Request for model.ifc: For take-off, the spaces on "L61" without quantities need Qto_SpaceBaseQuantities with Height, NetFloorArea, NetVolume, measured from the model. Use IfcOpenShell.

First a look at what the model holds.

```python
import ifcopenshell
import ifcopenshell.util.element
import ifcopenshell.util.unit

model = ifcopenshell.open("model.ifc")
print(model.schema)
for unit_type in ("LENGTHUNIT", "AREAUNIT", "VOLUMEUNIT"):
    print(unit_type, ifcopenshell.util.unit.calculate_unit_scale(model, unit_type))
storey = next(s for s in model.by_type("IfcBuildingStorey") if s.Name == "L61")
spaces = [e for e in ifcopenshell.util.element.get_decomposition(storey) if e.is_a("IfcSpace")]
for e in sorted(spaces, key=lambda e: e.id()):
    print(e.id(), e.is_a(), e.Name, list(ifcopenshell.util.element.get_psets(e, qtos_only=True)), sep=" | ")
```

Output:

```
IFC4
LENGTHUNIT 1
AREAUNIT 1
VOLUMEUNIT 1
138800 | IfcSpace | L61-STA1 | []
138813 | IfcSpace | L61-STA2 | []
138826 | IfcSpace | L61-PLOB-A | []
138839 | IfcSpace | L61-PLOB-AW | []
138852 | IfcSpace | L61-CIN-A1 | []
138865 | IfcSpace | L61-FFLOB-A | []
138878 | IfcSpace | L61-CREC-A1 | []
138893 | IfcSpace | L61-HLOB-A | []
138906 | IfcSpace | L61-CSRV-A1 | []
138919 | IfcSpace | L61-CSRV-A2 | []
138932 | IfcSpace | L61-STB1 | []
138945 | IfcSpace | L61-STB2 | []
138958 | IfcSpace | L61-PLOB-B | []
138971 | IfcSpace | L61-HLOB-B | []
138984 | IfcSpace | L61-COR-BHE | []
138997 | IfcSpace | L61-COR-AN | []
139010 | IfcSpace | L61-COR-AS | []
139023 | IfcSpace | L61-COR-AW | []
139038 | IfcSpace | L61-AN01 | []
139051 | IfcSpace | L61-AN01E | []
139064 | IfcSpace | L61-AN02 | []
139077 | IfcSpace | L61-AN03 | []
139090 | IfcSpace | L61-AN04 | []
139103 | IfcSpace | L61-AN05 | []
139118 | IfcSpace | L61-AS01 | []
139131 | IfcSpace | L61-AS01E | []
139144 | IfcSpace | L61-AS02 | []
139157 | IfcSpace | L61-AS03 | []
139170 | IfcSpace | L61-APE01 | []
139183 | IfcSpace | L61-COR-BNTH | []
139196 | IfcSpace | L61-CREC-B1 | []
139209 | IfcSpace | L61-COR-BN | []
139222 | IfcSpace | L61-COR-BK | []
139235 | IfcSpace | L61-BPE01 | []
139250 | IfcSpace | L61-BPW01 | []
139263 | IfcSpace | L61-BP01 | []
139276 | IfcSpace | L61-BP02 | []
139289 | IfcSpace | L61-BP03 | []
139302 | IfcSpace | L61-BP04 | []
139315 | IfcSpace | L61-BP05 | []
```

```python
import ifcopenshell
import ifcopenshell.api.pset
import ifcopenshell.geom
import ifcopenshell.util.element
import ifcopenshell.util.shape
import ifcopenshell.util.unit

model = ifcopenshell.open("model.ifc")
unit_scale = ifcopenshell.util.unit.calculate_unit_scale(model)
area_scale = ifcopenshell.util.unit.calculate_unit_scale(model, "AREAUNIT")
volume_scale = ifcopenshell.util.unit.calculate_unit_scale(model, "VOLUMEUNIT")
settings = ifcopenshell.geom.settings()

storey = next(s for s in model.by_type("IfcBuildingStorey") if s.Name == "L61")
spaces = [e for e in ifcopenshell.util.element.get_decomposition(storey) if e.is_a("IfcSpace")]

for e in sorted(spaces, key=lambda e: e.id()):
    if ifcopenshell.util.element.get_psets(e, qtos_only=True, should_inherit=False):
        continue
    # Geometry comes back in metres, in the element's own axes.
    shape = ifcopenshell.geom.create_shape(settings, e)
    values = {
        "Height": ifcopenshell.util.shape.get_z(shape.geometry) / unit_scale,
        "NetFloorArea": ifcopenshell.util.shape.get_footprint_area(shape.geometry) / area_scale,
        "NetVolume": ifcopenshell.util.shape.get_volume(shape.geometry) / volume_scale,
    }
    qto = ifcopenshell.api.pset.add_qto(model, product=e, name="Qto_SpaceBaseQuantities")
    ifcopenshell.api.pset.edit_qto(model, qto=qto, properties=values)
    print(e.id(), {k: round(v, 3) for k, v in values.items()})

model.write("model_rev.ifc")
```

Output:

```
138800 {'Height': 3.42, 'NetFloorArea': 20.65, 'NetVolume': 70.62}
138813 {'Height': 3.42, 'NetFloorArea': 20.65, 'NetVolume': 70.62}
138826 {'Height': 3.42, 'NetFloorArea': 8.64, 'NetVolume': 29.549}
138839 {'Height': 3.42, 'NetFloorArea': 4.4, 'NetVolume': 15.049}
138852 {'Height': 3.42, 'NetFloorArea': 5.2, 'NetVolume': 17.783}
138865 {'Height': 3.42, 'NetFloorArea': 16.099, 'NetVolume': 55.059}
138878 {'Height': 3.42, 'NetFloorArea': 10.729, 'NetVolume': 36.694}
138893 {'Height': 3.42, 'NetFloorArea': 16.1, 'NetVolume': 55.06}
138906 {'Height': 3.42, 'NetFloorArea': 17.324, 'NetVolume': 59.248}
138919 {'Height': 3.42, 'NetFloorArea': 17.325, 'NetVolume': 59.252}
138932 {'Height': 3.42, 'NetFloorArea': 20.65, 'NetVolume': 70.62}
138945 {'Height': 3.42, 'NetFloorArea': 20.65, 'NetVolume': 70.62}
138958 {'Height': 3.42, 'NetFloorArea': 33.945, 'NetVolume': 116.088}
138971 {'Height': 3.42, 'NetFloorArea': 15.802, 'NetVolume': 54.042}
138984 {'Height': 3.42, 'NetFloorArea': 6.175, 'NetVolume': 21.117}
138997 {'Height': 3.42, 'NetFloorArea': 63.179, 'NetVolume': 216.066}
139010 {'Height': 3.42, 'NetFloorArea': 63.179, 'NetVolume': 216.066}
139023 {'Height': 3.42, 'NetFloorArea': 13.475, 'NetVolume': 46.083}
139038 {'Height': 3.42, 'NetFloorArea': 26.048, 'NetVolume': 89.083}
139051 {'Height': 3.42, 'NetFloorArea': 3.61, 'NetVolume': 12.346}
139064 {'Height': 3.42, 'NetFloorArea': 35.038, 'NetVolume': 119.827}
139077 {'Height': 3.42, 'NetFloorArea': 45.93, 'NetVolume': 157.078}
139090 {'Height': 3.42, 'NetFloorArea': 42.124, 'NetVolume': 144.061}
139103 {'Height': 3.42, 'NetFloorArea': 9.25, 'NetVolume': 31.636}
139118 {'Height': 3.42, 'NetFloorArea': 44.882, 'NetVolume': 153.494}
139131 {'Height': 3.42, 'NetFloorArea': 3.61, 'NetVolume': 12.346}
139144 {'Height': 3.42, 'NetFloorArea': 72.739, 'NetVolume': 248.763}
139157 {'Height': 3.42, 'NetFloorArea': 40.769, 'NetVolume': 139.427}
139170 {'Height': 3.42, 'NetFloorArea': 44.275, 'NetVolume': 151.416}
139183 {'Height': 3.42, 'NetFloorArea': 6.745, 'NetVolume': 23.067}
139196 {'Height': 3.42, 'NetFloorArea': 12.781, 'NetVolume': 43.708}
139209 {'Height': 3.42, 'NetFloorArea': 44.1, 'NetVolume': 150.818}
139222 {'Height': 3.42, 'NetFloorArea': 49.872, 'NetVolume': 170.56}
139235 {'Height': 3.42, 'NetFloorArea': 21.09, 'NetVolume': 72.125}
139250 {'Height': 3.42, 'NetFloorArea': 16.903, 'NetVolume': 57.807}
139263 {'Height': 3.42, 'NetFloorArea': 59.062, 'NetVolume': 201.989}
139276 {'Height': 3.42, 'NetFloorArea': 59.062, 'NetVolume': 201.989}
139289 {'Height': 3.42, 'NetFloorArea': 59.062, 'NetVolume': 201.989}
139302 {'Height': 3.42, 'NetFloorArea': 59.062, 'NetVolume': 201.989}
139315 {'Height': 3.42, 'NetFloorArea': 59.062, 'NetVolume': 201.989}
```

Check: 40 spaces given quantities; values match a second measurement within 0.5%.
